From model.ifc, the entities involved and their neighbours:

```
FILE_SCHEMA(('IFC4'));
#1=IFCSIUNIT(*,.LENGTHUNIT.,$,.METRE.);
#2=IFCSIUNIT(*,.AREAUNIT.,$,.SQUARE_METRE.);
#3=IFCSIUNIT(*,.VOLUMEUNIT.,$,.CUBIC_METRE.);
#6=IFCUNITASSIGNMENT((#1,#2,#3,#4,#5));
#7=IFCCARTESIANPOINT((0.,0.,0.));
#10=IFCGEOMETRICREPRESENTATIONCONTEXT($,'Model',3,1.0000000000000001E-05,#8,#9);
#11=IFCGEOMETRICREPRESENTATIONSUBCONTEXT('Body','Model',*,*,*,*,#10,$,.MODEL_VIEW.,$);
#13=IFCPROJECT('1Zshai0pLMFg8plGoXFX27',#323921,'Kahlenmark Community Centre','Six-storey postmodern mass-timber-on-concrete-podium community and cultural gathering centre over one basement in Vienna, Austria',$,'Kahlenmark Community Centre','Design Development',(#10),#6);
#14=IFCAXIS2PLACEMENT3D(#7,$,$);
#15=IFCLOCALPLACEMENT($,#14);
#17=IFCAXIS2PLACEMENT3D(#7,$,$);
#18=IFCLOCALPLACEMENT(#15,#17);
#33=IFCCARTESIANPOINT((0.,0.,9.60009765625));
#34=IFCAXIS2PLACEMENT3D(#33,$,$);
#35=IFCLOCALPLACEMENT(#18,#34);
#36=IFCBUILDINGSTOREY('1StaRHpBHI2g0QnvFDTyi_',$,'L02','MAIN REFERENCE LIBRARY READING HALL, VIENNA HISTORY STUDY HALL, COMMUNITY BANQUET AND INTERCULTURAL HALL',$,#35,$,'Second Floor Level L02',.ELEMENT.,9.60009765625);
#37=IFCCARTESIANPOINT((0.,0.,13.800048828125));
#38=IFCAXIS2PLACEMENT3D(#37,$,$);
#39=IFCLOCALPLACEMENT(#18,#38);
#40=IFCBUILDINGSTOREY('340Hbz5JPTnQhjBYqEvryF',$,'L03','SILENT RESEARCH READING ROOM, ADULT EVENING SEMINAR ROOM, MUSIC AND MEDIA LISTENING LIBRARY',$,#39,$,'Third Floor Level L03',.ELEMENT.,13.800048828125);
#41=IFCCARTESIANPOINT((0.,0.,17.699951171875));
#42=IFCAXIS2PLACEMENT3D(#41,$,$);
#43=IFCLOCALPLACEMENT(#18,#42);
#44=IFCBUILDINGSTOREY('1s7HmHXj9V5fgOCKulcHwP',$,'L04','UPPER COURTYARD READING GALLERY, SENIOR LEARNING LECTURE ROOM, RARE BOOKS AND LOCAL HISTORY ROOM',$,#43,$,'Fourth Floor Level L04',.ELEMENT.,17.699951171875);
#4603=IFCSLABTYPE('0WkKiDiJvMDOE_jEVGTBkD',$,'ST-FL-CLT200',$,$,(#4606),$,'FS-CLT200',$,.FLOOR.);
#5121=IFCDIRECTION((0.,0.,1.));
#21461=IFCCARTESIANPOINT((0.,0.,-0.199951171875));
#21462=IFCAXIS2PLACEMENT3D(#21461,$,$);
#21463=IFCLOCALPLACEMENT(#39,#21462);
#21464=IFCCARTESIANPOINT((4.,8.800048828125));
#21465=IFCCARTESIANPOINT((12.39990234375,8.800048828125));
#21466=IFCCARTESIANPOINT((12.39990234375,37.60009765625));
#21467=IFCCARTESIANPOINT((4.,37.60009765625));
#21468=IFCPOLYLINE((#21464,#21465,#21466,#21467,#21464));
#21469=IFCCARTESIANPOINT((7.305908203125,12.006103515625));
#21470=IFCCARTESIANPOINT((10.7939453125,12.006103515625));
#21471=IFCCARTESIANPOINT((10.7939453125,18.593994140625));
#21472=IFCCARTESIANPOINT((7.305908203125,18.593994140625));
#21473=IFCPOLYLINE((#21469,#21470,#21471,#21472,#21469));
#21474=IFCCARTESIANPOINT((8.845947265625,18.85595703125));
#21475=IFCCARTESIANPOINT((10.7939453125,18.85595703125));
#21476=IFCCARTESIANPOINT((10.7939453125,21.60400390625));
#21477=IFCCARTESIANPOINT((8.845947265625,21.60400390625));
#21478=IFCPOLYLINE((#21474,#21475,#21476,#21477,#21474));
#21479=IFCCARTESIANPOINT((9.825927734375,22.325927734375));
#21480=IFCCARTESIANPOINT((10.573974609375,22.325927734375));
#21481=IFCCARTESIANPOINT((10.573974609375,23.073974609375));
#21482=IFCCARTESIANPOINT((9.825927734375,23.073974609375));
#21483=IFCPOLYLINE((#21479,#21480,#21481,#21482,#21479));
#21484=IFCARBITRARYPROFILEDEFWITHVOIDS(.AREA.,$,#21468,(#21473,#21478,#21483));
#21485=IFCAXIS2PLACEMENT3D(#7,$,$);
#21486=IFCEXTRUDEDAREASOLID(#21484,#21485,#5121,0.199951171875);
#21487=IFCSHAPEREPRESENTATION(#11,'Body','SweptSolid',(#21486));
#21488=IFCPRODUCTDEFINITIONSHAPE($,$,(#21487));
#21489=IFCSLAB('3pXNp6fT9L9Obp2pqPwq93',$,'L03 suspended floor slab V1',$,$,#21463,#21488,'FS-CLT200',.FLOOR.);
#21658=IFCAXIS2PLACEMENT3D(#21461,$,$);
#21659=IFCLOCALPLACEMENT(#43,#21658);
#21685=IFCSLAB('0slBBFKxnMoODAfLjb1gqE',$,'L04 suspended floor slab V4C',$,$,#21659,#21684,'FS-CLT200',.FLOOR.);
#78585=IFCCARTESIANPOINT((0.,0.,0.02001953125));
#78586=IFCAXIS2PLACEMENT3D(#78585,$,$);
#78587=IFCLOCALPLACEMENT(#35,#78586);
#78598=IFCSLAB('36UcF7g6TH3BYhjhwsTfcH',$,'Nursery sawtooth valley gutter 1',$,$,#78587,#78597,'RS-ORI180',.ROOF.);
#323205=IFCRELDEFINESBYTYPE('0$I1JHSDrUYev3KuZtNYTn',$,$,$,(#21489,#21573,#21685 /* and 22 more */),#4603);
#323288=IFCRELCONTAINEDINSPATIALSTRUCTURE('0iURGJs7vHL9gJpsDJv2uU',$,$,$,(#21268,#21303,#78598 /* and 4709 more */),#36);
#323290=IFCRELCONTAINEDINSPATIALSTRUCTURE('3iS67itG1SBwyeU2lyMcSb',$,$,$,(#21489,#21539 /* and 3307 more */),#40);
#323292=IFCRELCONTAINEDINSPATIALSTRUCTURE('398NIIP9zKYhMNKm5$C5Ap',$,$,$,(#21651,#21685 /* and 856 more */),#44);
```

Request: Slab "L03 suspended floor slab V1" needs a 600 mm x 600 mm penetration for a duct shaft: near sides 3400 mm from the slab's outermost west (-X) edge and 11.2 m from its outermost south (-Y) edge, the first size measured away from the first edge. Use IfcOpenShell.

```python
import numpy as np
import ifcopenshell
import ifcopenshell.api.feature
import ifcopenshell.api.geometry
import ifcopenshell.api.root
import ifcopenshell.geom
import ifcopenshell.util.placement
import ifcopenshell.util.representation
import ifcopenshell.util.shape
import ifcopenshell.util.unit

model = ifcopenshell.open("model.ifc")
unit_scale = ifcopenshell.util.unit.calculate_unit_scale(model)
settings = ifcopenshell.geom.settings()


def volume(element):
    """Net volume in cubic metres, openings subtracted."""
    shape = ifcopenshell.geom.create_shape(settings, element)
    return ifcopenshell.util.shape.get_volume(shape.geometry)


slab = model.by_guid("3pXNp6fT9L9Obp2pqPwq93")
before = volume(slab)

# Extent in the slab's own axes, in metres. The edges named are its -X and -Y sides.
slab_shape = ifcopenshell.geom.create_shape(settings, slab)
vertices = ifcopenshell.util.shape.get_vertices(slab_shape.geometry)
x_min, y_min, bottom = vertices.min(axis=0)
top = vertices[:, 2].max()

opening = ifcopenshell.api.root.create_entity(model, ifc_class="IfcOpeningElement", name="Duct shaft opening", predefined_type="OPENING")
context = ifcopenshell.util.representation.get_context(model, "Model", "Body", "MODEL_VIEW")
width, depth = 0.6, 0.6
outline = [(0.0, 0.0), (width, 0.0), (width, depth), (0.0, depth), (0.0, 0.0)]
# Overshoot both faces by 50 mm so the cut is clean.
shape = ifcopenshell.api.geometry.add_slab_representation(
    model, context=context, depth=top - bottom + 0.1, polyline=outline
)
ifcopenshell.api.geometry.assign_representation(model, product=opening, representation=shape)

matrix = ifcopenshell.util.placement.get_local_placement(slab.ObjectPlacement)
matrix[:, 3] = matrix @ np.append(np.array([x_min + 3.4, y_min + 11.2, bottom - 0.05]) / unit_scale, 1.0)
ifcopenshell.api.geometry.edit_object_placement(model, product=opening, matrix=matrix, is_si=False)
ifcopenshell.api.feature.add_feature(model, feature=opening, element=slab)

after = volume(slab)

print(f"slab volume {before:.3f} -> {after:.3f} m3")

model.write("model_rev.ifc")
```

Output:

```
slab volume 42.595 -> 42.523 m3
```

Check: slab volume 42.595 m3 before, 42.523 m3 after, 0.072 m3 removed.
